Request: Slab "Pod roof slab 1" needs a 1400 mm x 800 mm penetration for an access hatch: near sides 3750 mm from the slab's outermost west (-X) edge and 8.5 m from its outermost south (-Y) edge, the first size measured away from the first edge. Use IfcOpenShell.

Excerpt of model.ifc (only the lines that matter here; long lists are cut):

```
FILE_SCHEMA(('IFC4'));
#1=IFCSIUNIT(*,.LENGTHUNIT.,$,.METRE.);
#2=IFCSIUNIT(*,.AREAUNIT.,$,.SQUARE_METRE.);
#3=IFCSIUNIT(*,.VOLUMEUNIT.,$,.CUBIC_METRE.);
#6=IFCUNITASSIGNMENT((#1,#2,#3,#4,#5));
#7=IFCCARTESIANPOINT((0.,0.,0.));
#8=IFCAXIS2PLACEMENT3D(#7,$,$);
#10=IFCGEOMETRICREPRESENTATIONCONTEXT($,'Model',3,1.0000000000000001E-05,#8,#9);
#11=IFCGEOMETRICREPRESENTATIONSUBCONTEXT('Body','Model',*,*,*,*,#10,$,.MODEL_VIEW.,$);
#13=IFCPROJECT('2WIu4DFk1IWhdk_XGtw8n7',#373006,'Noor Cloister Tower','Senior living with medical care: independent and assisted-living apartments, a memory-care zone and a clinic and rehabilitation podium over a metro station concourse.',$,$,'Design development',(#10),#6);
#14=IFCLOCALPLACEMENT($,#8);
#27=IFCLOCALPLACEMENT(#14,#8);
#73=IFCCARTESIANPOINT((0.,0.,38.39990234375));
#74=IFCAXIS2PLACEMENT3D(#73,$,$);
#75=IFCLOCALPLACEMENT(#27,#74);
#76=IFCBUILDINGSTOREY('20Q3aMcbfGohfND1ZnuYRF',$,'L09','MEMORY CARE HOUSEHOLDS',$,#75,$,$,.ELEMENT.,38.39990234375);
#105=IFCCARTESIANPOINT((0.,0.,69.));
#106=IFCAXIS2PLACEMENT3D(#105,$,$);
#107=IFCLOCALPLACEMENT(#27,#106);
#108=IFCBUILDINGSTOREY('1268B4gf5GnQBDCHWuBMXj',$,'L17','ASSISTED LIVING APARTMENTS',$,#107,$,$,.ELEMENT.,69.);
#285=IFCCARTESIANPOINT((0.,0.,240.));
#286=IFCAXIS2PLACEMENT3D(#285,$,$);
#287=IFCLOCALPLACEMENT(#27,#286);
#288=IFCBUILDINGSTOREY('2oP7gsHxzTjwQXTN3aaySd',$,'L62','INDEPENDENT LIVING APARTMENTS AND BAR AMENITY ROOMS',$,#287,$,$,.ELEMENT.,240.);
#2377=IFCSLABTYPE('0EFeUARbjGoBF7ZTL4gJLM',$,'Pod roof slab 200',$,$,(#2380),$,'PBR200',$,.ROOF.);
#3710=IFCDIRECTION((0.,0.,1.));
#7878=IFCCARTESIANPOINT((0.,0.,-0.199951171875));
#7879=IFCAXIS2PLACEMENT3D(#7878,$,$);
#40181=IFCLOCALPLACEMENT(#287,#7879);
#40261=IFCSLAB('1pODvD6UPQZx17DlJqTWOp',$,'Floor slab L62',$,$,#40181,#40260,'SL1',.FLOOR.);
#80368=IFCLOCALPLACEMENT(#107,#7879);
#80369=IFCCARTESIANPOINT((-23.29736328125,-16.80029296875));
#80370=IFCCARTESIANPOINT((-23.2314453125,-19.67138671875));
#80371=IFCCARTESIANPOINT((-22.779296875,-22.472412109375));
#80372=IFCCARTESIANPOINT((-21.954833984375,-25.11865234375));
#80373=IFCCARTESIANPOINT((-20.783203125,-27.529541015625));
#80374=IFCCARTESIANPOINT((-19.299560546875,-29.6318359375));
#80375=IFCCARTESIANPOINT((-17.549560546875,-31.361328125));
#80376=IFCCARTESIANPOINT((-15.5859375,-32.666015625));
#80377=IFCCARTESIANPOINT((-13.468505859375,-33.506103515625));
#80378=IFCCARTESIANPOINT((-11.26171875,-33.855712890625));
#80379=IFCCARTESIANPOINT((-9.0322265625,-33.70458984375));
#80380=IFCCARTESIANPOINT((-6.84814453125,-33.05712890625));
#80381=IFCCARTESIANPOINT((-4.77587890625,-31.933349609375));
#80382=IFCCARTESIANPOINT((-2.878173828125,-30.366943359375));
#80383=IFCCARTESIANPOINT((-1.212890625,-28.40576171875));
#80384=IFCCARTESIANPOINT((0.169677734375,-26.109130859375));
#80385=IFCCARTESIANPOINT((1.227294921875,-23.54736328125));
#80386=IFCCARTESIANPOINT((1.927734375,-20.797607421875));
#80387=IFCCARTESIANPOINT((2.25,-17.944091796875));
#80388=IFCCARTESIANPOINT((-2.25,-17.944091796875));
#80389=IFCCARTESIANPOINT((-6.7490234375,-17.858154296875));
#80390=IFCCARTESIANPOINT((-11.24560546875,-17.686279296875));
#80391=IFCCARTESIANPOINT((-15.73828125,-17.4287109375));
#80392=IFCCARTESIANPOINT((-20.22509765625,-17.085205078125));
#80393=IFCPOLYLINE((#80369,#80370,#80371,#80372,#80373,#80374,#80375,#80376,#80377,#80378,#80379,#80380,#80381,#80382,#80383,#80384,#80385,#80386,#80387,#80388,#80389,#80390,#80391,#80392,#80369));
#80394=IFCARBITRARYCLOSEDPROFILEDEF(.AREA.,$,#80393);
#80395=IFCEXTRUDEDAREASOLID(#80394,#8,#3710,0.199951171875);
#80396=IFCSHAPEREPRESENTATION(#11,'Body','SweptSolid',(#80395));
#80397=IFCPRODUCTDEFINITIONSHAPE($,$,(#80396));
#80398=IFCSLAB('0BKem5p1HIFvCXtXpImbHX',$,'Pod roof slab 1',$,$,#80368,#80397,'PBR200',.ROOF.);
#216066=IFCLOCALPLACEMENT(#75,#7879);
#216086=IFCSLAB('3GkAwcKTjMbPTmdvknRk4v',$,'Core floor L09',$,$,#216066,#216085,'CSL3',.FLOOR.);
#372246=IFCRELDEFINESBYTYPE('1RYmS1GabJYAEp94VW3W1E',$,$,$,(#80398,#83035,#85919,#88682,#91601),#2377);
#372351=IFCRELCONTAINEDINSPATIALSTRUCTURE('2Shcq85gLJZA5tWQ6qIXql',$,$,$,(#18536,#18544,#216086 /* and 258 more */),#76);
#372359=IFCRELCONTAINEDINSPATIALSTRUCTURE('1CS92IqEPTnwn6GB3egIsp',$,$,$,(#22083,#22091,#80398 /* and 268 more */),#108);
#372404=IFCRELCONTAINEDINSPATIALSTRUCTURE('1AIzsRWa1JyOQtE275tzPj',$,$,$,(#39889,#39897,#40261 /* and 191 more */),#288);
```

```python
import numpy as np
import ifcopenshell
import ifcopenshell.api.feature
import ifcopenshell.api.geometry
import ifcopenshell.api.root
import ifcopenshell.geom
import ifcopenshell.util.placement
import ifcopenshell.util.representation
import ifcopenshell.util.shape
import ifcopenshell.util.unit

model = ifcopenshell.open("model.ifc")
unit_scale = ifcopenshell.util.unit.calculate_unit_scale(model)
settings = ifcopenshell.geom.settings()


def volume(element):
    """Net volume in cubic metres, openings subtracted."""
    shape = ifcopenshell.geom.create_shape(settings, element)
    return ifcopenshell.util.shape.get_volume(shape.geometry)


slab = model.by_id(80398)
before = volume(slab)

# Extent in the slab's own axes, in metres. The edges named are its -X and -Y sides.
slab_shape = ifcopenshell.geom.create_shape(settings, slab)
vertices = ifcopenshell.util.shape.get_vertices(slab_shape.geometry)
x_min, y_min, bottom = vertices.min(axis=0)
top = vertices[:, 2].max()

opening = ifcopenshell.api.root.create_entity(model, ifc_class="IfcOpeningElement", name="Access hatch opening", predefined_type="OPENING")
context = ifcopenshell.util.representation.get_context(model, "Model", "Body", "MODEL_VIEW")
width, depth = 1.4, 0.8
outline = [(0.0, 0.0), (width, 0.0), (width, depth), (0.0, depth), (0.0, 0.0)]
# Overshoot both faces by 50 mm so the cut is clean.
shape = ifcopenshell.api.geometry.add_slab_representation(
    model, context=context, depth=top - bottom + 0.1, polyline=outline
)
ifcopenshell.api.geometry.assign_representation(model, product=opening, representation=shape)

matrix = ifcopenshell.util.placement.get_local_placement(slab.ObjectPlacement)
matrix[:, 3] = matrix @ np.append(np.array([x_min + 3.75, y_min + 8.5, bottom - 0.05]) / unit_scale, 1.0)
ifcopenshell.api.geometry.edit_object_placement(model, product=opening, matrix=matrix, is_si=False)
ifcopenshell.api.feature.add_feature(model, feature=opening, element=slab)

after = volume(slab)

print(f"slab volume {before:.3f} -> {after:.3f} m3")

model.write("model_edited.ifc")
```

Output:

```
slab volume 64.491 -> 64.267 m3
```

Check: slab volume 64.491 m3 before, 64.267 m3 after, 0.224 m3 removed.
